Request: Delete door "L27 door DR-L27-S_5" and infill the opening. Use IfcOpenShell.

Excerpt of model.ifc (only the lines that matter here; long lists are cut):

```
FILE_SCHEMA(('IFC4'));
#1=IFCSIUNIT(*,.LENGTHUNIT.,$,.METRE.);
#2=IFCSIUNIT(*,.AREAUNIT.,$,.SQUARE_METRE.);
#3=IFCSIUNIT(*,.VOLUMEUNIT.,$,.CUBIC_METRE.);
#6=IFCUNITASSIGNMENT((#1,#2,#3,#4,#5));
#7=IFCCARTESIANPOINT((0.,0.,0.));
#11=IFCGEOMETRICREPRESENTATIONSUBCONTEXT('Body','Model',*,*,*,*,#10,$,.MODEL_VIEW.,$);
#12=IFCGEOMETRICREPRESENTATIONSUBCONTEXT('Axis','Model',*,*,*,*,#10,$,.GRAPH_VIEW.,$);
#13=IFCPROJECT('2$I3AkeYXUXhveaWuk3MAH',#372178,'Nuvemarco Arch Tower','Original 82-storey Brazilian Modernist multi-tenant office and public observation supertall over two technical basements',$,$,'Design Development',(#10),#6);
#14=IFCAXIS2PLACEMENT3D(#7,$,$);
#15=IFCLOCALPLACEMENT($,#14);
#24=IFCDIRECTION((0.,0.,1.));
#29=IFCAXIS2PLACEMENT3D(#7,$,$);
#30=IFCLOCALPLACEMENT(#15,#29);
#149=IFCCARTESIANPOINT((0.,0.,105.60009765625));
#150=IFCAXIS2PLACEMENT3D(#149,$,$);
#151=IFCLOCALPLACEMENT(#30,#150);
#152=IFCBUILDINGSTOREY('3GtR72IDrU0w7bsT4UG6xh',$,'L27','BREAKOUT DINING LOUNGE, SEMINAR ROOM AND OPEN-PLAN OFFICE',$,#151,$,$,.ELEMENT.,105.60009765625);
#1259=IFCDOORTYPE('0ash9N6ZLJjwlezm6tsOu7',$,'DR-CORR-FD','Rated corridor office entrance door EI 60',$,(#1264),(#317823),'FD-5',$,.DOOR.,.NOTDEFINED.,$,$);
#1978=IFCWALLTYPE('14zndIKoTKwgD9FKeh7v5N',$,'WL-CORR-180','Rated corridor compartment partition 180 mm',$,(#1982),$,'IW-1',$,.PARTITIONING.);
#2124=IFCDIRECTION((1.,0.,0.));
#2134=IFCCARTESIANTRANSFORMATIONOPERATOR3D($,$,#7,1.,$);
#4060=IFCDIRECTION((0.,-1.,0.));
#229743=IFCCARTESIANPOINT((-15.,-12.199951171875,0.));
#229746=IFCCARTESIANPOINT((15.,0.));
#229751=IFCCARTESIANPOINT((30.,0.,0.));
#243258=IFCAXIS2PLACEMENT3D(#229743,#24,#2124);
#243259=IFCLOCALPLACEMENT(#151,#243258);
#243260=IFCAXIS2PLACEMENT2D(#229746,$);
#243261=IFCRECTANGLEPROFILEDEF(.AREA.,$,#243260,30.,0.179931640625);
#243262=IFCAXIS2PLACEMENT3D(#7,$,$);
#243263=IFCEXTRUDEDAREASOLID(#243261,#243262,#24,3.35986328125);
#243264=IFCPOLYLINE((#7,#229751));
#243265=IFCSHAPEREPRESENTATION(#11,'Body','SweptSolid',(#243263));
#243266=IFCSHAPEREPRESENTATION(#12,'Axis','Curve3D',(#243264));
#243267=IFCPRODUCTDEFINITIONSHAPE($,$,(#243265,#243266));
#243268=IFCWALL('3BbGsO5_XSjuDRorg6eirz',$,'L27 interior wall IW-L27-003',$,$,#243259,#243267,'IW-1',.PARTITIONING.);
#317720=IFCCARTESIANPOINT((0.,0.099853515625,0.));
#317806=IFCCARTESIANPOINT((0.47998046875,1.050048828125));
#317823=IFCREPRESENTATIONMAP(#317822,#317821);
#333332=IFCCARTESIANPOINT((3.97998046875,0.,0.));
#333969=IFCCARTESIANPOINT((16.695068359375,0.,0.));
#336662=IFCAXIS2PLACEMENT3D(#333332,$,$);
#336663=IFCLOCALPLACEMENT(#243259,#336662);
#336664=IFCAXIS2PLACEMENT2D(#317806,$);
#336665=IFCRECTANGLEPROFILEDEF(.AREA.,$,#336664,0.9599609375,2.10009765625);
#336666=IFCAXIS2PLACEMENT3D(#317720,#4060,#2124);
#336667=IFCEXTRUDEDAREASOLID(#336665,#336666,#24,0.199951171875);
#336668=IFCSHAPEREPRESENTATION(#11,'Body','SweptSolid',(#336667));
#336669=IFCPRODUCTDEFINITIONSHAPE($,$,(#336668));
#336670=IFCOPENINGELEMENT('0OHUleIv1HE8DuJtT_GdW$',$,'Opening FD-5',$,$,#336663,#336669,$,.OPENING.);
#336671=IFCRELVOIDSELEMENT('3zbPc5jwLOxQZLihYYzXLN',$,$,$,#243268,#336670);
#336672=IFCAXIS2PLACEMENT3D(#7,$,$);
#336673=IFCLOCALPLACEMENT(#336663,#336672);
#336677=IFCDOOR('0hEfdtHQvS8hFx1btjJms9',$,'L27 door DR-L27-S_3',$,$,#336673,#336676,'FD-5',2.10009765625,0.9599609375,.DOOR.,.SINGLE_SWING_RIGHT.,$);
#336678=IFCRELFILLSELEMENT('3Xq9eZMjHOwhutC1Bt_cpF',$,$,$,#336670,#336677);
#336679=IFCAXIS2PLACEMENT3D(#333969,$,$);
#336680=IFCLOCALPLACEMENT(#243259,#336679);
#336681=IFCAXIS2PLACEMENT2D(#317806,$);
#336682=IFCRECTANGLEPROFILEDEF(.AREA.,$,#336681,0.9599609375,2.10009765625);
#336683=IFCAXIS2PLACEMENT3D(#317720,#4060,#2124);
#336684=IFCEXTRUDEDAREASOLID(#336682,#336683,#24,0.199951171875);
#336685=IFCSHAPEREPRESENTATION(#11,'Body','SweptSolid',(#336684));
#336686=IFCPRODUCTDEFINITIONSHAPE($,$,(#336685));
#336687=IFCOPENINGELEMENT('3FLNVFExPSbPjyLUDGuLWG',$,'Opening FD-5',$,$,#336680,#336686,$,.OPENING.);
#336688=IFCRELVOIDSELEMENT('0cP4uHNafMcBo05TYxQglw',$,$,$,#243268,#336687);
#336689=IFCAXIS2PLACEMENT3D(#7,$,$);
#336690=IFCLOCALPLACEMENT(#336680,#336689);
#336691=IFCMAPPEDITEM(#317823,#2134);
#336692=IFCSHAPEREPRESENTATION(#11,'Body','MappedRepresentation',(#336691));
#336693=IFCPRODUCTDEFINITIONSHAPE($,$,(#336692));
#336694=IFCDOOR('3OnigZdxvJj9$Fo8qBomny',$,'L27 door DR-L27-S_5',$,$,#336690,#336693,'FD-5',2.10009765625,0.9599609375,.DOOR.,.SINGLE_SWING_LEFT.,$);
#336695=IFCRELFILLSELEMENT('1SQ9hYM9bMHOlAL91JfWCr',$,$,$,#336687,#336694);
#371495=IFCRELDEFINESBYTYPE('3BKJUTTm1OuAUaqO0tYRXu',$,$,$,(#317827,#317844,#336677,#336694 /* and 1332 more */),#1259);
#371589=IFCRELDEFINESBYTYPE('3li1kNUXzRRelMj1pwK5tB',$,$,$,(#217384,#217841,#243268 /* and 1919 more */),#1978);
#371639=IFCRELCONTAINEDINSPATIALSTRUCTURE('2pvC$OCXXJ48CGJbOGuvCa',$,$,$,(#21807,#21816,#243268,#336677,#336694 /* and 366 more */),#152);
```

```python
import ifcopenshell
import ifcopenshell.api.feature
import ifcopenshell.api.root
import ifcopenshell.geom
import ifcopenshell.util.shape

model = ifcopenshell.open("model.ifc")
settings = ifcopenshell.geom.settings()


def volume(element):
    """Net volume in cubic metres, openings subtracted."""
    shape = ifcopenshell.geom.create_shape(settings, element)
    return ifcopenshell.util.shape.get_volume(shape.geometry)


door = model.by_guid("3OnigZdxvJj9$Fo8qBomny")
opening = door.FillsVoids[0].RelatingOpeningElement
wall = opening.VoidsElements[0].RelatingBuildingElement
before = volume(wall)

ifcopenshell.api.root.remove_product(model, product=door)
ifcopenshell.api.feature.remove_feature(model, feature=opening)

after = volume(wall)

print(f"wall volume {before:.3f} -> {after:.3f} m3")

model.write("model_rev.ifc")
```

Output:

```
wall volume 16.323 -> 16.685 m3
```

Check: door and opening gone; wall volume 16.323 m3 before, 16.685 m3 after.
